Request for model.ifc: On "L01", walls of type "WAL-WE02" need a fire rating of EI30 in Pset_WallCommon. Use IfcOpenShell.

First a look at what the model holds.

```python
import ifcopenshell
import ifcopenshell.util.element

model = ifcopenshell.open("model.ifc")
print(model.schema)
storey = next(s for s in model.by_type("IfcBuildingStorey") if s.Name == "L01")
walls = [e for e in ifcopenshell.util.element.get_decomposition(storey) if e.is_a("IfcWall")]
seen = {}
for e in walls:
    element_type = ifcopenshell.util.element.get_type(e)
    key = (element_type.Name if element_type != e and element_type else None, ifcopenshell.util.element.get_pset(e, "Pset_WallCommon", "FireRating"))
    seen[key] = seen.get(key, 0) + 1
for (name, value), count in sorted(seen.items(), key=str):
    print(count, "x", name, "|", value)
```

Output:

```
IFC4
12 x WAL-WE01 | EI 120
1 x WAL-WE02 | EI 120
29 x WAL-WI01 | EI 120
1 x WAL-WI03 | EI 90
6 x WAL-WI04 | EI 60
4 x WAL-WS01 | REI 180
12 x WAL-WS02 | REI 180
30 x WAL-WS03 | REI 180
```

```python
import ifcopenshell
import ifcopenshell.api.pset
import ifcopenshell.util.element

model = ifcopenshell.open("model.ifc")

storey = next(s for s in model.by_type("IfcBuildingStorey") if s.Name == "L01")
walls = [e for e in ifcopenshell.util.element.get_decomposition(storey) if e.is_a("IfcWall")]

count = 0
for e in walls:
    element_type = ifcopenshell.util.element.get_type(e)
    if element_type in (None, e) or element_type.Name != "WAL-WE02":
        continue
    # add_pset returns the element's existing set when there is one.
    pset = ifcopenshell.api.pset.add_pset(model, product=e, name="Pset_WallCommon")
    ifcopenshell.api.pset.edit_pset(model, pset=pset, properties={"FireRating": "EI30"})
    count += 1

print(count, "walls updated")

model.write("model-out.ifc")
```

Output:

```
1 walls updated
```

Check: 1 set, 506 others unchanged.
